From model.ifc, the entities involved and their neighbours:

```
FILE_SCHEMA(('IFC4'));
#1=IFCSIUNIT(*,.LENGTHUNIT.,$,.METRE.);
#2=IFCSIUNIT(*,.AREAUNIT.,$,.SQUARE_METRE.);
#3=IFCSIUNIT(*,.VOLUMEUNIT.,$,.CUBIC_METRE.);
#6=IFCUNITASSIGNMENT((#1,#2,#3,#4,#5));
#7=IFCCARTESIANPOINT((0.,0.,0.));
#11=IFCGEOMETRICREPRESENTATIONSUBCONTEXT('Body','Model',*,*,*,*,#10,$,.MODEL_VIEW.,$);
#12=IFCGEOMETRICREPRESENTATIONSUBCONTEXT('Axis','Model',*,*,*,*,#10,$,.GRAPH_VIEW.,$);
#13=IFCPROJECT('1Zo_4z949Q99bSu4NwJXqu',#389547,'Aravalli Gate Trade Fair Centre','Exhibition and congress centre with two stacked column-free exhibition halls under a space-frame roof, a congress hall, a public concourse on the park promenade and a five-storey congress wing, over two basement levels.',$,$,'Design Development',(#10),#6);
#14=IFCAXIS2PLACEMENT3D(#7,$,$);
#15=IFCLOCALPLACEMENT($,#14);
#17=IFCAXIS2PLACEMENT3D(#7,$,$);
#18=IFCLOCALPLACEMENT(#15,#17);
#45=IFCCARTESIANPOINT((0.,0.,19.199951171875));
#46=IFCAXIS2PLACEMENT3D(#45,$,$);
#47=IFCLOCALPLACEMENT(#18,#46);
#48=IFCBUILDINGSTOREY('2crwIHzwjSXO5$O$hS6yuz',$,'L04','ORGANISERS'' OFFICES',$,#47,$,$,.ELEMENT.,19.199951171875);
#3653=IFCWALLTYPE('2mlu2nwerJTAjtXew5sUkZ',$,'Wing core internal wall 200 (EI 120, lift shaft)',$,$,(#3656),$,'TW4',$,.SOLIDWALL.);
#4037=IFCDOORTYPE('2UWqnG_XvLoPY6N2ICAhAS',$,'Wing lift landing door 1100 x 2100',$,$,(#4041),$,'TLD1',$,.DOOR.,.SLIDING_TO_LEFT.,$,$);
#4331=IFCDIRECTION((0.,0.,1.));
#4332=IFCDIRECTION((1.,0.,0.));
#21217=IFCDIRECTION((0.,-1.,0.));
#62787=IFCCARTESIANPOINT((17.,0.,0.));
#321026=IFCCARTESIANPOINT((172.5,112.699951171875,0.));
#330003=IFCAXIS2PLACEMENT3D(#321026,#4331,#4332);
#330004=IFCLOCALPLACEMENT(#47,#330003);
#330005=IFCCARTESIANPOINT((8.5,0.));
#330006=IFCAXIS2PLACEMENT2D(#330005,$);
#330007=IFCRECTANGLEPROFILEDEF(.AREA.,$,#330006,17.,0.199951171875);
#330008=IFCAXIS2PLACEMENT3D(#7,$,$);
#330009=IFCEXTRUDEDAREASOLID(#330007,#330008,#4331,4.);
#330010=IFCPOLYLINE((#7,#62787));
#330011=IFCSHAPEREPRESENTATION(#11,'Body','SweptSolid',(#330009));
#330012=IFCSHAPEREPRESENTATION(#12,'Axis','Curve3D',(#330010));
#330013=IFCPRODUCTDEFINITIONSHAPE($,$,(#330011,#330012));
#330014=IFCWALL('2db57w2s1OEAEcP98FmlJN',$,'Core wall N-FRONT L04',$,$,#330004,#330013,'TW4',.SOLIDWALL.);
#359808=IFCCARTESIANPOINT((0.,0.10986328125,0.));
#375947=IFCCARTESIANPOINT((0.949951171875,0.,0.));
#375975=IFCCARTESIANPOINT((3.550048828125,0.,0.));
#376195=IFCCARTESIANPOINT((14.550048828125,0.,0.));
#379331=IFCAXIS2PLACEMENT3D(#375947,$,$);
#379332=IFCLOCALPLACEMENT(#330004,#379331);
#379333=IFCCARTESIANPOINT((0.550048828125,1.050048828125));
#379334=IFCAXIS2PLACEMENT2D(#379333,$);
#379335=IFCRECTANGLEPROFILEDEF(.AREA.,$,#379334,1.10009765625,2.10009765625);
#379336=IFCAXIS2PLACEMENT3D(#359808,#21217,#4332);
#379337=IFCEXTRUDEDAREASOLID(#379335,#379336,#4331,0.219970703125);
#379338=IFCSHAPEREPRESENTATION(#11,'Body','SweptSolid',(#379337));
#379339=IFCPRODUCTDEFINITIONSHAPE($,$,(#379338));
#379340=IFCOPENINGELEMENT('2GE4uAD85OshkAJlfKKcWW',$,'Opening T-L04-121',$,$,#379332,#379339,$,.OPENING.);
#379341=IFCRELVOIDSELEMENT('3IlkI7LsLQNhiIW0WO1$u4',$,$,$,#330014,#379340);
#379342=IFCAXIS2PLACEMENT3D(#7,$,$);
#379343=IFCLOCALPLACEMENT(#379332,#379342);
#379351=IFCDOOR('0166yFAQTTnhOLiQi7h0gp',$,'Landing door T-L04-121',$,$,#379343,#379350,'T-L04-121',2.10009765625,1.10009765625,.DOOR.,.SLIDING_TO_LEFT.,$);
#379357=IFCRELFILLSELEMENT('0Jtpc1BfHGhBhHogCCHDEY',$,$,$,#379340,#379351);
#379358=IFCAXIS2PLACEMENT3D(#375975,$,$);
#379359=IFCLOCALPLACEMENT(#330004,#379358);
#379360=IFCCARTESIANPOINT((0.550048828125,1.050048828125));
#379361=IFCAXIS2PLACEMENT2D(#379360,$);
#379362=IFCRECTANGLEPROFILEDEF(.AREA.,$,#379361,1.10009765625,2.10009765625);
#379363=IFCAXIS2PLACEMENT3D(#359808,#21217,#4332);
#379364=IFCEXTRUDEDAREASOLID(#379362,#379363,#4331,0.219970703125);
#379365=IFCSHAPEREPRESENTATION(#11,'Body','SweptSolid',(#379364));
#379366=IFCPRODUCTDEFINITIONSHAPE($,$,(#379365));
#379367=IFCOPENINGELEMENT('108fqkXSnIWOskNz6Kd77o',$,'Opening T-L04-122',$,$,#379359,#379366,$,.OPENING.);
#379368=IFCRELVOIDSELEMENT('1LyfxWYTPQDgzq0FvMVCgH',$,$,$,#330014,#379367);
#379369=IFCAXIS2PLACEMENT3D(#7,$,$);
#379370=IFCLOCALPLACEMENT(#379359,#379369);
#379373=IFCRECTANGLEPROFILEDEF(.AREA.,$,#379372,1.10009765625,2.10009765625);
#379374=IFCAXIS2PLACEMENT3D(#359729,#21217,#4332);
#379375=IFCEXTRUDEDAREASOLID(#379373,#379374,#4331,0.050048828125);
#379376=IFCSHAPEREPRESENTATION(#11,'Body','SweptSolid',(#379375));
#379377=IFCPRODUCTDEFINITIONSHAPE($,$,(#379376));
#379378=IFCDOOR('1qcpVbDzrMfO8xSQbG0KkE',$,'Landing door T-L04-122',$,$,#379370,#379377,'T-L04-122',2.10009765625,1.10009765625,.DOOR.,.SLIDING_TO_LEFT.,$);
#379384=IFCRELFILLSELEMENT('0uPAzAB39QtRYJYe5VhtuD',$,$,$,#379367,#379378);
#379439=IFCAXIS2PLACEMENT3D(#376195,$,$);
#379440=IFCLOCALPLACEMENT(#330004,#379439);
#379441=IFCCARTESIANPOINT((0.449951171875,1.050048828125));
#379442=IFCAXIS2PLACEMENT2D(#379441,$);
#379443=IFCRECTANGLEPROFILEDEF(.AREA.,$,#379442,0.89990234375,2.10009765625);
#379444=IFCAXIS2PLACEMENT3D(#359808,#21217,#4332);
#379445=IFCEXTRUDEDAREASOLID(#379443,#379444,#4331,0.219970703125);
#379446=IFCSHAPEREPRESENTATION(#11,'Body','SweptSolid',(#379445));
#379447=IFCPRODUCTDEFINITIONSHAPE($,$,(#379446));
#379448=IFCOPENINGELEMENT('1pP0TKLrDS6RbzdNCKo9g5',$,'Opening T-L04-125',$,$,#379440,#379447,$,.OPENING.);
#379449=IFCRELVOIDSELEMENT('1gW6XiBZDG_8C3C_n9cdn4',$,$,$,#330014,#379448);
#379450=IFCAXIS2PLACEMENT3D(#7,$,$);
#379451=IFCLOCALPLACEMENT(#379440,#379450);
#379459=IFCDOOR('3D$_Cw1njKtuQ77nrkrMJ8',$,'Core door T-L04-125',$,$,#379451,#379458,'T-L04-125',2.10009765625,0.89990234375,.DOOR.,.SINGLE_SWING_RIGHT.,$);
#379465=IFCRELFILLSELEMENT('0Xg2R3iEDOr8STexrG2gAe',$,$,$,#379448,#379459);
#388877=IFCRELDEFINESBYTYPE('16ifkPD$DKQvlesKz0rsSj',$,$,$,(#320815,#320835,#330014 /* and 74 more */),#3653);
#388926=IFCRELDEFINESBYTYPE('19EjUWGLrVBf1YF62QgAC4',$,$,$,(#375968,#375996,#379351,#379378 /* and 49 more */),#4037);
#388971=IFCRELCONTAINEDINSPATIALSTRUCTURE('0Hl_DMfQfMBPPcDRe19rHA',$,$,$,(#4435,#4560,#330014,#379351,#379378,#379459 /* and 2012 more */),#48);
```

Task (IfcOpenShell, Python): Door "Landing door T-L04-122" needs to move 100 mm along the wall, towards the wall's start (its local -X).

```python
import ifcopenshell
import ifcopenshell.api.geometry
import ifcopenshell.util.placement
import ifcopenshell.util.unit

model = ifcopenshell.open("model.ifc")
unit_scale = ifcopenshell.util.unit.calculate_unit_scale(model)

door = model.by_guid("1qcpVbDzrMfO8xSQbG0KkE")
opening = door.FillsVoids[0].RelatingOpeningElement
wall = opening.VoidsElements[0].RelatingBuildingElement

wall_matrix = ifcopenshell.util.placement.get_local_placement(wall.ObjectPlacement)
shift = wall_matrix[:3, 0] * -0.1 / unit_scale
before = ifcopenshell.util.placement.get_local_placement(door.ObjectPlacement)[:3, 3].copy()

# The door is placed relative to its opening, so it follows when the opening moves.
matrix = ifcopenshell.util.placement.get_local_placement(opening.ObjectPlacement)
matrix[:3, 3] += shift
ifcopenshell.api.geometry.edit_object_placement(
    model, product=opening, matrix=matrix, is_si=False, should_transform_children=True
)

after = ifcopenshell.util.placement.get_local_placement(door.ObjectPlacement)[:3, 3]
print("door moved by", (after - before).round(3) + 0.0)

model.write("model_v2.ifc")
```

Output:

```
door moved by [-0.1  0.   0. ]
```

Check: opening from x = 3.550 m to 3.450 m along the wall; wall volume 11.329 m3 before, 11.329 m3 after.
